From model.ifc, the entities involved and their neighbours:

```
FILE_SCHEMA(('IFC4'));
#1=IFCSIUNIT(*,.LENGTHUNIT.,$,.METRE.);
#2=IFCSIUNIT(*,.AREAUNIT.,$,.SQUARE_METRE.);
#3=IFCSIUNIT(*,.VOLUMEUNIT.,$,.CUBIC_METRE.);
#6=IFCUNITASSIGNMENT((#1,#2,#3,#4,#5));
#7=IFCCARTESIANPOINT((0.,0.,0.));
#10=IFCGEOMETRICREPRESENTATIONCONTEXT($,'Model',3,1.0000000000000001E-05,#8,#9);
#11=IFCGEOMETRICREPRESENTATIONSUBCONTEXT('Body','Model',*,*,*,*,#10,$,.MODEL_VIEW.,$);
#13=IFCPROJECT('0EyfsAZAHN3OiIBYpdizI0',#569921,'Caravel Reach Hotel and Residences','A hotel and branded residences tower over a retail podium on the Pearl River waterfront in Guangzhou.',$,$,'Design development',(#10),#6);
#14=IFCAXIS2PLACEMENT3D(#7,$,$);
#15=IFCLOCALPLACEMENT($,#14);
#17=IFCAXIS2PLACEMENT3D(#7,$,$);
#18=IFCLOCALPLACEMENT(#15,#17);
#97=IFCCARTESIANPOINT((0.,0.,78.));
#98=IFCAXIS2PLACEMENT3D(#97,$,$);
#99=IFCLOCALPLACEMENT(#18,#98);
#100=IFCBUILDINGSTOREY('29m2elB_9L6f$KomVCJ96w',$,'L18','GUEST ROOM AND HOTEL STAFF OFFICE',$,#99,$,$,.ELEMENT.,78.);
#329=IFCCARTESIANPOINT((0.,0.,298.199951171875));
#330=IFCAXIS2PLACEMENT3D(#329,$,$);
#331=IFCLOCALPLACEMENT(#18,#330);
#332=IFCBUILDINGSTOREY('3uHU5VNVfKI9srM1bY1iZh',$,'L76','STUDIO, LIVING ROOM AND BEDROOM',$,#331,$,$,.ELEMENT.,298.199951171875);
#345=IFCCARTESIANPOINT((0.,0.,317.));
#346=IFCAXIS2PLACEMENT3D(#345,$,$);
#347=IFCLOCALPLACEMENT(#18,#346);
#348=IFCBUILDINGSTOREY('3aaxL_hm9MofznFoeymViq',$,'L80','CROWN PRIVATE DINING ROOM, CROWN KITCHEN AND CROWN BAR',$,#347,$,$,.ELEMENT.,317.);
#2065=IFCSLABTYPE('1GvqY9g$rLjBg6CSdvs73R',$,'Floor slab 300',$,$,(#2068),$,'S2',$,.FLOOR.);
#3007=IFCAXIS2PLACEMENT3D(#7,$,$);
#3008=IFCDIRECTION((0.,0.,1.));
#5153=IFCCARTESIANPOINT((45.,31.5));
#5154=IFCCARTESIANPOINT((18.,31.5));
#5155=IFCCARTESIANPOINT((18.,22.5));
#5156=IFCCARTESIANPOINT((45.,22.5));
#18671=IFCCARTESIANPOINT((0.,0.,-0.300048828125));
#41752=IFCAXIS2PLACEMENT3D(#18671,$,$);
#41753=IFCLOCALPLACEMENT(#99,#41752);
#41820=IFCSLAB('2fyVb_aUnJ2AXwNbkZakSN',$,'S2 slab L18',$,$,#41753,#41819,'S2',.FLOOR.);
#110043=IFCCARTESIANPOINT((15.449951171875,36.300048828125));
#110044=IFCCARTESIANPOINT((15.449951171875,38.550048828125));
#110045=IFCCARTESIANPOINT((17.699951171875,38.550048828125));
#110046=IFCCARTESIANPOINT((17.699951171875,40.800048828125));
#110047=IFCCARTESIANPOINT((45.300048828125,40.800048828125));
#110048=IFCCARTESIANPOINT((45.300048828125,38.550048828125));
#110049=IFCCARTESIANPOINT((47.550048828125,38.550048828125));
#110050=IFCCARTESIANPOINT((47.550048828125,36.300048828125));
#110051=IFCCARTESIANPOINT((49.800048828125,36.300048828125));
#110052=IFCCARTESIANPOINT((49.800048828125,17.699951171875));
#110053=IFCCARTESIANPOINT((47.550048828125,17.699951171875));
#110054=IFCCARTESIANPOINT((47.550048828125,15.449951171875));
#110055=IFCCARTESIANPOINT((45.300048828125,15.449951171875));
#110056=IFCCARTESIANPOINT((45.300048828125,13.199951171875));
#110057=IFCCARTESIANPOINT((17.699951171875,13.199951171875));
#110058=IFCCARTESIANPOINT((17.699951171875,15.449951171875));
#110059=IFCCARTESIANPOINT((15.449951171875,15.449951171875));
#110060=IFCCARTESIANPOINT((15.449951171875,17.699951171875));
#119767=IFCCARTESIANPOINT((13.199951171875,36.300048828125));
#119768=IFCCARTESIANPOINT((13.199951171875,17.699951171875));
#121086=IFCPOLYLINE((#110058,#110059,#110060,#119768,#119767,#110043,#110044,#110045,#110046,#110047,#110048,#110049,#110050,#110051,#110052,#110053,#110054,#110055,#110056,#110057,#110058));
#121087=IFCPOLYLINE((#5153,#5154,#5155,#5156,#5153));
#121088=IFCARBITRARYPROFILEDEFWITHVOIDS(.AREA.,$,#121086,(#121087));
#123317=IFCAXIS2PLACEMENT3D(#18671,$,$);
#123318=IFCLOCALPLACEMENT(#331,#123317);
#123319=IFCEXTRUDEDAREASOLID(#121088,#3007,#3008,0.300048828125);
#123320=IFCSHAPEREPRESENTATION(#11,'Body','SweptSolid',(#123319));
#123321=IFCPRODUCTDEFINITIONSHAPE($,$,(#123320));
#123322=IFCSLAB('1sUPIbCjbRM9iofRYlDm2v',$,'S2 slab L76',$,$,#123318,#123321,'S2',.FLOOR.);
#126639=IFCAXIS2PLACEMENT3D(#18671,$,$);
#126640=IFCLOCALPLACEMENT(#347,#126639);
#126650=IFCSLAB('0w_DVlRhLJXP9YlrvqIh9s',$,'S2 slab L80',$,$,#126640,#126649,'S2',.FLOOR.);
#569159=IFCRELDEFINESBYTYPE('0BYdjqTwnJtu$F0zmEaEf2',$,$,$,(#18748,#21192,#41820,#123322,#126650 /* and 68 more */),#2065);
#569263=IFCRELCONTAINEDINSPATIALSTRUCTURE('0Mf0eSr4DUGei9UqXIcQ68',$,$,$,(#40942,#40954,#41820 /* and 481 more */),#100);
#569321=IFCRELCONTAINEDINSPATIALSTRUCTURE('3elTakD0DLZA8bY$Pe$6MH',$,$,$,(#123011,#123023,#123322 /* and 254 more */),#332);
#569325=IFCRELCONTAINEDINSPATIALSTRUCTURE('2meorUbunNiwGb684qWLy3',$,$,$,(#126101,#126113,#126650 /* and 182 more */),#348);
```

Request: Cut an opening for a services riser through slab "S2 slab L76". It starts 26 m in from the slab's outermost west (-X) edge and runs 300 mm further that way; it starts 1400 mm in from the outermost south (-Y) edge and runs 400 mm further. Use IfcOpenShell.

```python
import numpy as np
import ifcopenshell
import ifcopenshell.api.feature
import ifcopenshell.api.geometry
import ifcopenshell.api.root
import ifcopenshell.geom
import ifcopenshell.util.placement
import ifcopenshell.util.representation
import ifcopenshell.util.shape
import ifcopenshell.util.unit

model = ifcopenshell.open("model.ifc")
unit_scale = ifcopenshell.util.unit.calculate_unit_scale(model)
settings = ifcopenshell.geom.settings()


def volume(element):
    """Net volume in cubic metres, openings subtracted."""
    shape = ifcopenshell.geom.create_shape(settings, element)
    return ifcopenshell.util.shape.get_volume(shape.geometry)


slab = model.by_guid("1sUPIbCjbRM9iofRYlDm2v")
before = volume(slab)

# Extent in the slab's own axes, in metres. The edges named are its -X and -Y sides.
slab_shape = ifcopenshell.geom.create_shape(settings, slab)
vertices = ifcopenshell.util.shape.get_vertices(slab_shape.geometry)
x_min, y_min, bottom = vertices.min(axis=0)
top = vertices[:, 2].max()

opening = ifcopenshell.api.root.create_entity(model, ifc_class="IfcOpeningElement", name="Services riser opening", predefined_type="OPENING")
context = ifcopenshell.util.representation.get_context(model, "Model", "Body", "MODEL_VIEW")
width, depth = 0.3, 0.4
outline = [(0.0, 0.0), (width, 0.0), (width, depth), (0.0, depth), (0.0, 0.0)]
# Overshoot both faces by 50 mm so the cut is clean.
shape = ifcopenshell.api.geometry.add_slab_representation(
    model, context=context, depth=top - bottom + 0.1, polyline=outline
)
ifcopenshell.api.geometry.assign_representation(model, product=opening, representation=shape)

matrix = ifcopenshell.util.placement.get_local_placement(slab.ObjectPlacement)
matrix[:, 3] = matrix @ np.append(np.array([x_min + 26, y_min + 1.4, bottom - 0.05]) / unit_scale, 1.0)
ifcopenshell.api.geometry.edit_object_placement(model, product=opening, matrix=matrix, is_si=False)
ifcopenshell.api.feature.add_feature(model, feature=opening, element=slab)

after = volume(slab)

print(f"slab volume {before:.3f} -> {after:.3f} m3")

model.write("model_v2.ifc")
```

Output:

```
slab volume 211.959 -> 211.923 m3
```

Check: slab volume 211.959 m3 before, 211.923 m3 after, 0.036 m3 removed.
